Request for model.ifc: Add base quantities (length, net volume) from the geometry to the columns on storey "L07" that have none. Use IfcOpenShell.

First a look at what the model holds.

```python
import ifcopenshell
import ifcopenshell.util.element
import ifcopenshell.util.unit

model = ifcopenshell.open("model.ifc")
print(model.schema)
for unit_type in ("LENGTHUNIT", "AREAUNIT", "VOLUMEUNIT"):
    print(unit_type, ifcopenshell.util.unit.calculate_unit_scale(model, unit_type))
storey = next(s for s in model.by_type("IfcBuildingStorey") if s.Name == "L07")
columns = [e for e in ifcopenshell.util.element.get_decomposition(storey) if e.is_a("IfcColumn")]
for e in sorted(columns, key=lambda e: e.id()):
    print(e.id(), e.is_a(), e.Name, list(ifcopenshell.util.element.get_psets(e, qtos_only=True)), sep=" | ")
```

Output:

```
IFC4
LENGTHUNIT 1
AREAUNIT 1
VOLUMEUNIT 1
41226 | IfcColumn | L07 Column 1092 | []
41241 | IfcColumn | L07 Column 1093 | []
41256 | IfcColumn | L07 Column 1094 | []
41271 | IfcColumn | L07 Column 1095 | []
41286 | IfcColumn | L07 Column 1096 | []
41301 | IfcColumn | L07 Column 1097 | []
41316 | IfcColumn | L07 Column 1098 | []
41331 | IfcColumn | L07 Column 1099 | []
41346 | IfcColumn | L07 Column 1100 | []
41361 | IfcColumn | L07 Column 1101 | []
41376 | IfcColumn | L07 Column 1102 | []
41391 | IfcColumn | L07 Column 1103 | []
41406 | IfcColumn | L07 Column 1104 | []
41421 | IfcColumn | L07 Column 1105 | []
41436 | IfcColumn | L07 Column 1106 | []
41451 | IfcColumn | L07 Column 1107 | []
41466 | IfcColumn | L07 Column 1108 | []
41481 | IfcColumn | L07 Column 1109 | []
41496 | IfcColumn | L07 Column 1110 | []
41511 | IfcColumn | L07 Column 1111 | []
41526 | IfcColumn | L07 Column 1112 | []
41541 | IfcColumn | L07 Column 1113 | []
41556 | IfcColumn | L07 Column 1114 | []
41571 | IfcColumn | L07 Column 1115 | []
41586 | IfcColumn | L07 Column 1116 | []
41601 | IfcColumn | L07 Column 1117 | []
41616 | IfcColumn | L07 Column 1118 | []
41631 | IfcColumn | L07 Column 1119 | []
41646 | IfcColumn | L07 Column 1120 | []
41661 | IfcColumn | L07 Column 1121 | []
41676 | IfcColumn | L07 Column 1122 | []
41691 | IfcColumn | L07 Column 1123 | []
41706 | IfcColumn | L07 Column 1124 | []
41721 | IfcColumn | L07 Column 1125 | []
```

```python
import ifcopenshell
import ifcopenshell.api.pset
import ifcopenshell.geom
import ifcopenshell.util.element
import ifcopenshell.util.shape
import ifcopenshell.util.unit

model = ifcopenshell.open("model.ifc")
unit_scale = ifcopenshell.util.unit.calculate_unit_scale(model)
volume_scale = ifcopenshell.util.unit.calculate_unit_scale(model, "VOLUMEUNIT")
settings = ifcopenshell.geom.settings()

storey = next(s for s in model.by_type("IfcBuildingStorey") if s.Name == "L07")
columns = [e for e in ifcopenshell.util.element.get_decomposition(storey) if e.is_a("IfcColumn")]

for e in sorted(columns, key=lambda e: e.id()):
    if ifcopenshell.util.element.get_psets(e, qtos_only=True, should_inherit=False):
        continue
    # Geometry comes back in metres, in the element's own axes.
    shape = ifcopenshell.geom.create_shape(settings, e)
    values = {
        "Length": ifcopenshell.util.shape.get_z(shape.geometry) / unit_scale,
        "NetVolume": ifcopenshell.util.shape.get_volume(shape.geometry) / volume_scale,
    }
    qto = ifcopenshell.api.pset.add_qto(model, product=e, name="Qto_ColumnBaseQuantities")
    ifcopenshell.api.pset.edit_qto(model, qto=qto, properties=values)
    print(e.id(), {k: round(v, 3) for k, v in values.items()})

model.write("model_edited.ifc")
```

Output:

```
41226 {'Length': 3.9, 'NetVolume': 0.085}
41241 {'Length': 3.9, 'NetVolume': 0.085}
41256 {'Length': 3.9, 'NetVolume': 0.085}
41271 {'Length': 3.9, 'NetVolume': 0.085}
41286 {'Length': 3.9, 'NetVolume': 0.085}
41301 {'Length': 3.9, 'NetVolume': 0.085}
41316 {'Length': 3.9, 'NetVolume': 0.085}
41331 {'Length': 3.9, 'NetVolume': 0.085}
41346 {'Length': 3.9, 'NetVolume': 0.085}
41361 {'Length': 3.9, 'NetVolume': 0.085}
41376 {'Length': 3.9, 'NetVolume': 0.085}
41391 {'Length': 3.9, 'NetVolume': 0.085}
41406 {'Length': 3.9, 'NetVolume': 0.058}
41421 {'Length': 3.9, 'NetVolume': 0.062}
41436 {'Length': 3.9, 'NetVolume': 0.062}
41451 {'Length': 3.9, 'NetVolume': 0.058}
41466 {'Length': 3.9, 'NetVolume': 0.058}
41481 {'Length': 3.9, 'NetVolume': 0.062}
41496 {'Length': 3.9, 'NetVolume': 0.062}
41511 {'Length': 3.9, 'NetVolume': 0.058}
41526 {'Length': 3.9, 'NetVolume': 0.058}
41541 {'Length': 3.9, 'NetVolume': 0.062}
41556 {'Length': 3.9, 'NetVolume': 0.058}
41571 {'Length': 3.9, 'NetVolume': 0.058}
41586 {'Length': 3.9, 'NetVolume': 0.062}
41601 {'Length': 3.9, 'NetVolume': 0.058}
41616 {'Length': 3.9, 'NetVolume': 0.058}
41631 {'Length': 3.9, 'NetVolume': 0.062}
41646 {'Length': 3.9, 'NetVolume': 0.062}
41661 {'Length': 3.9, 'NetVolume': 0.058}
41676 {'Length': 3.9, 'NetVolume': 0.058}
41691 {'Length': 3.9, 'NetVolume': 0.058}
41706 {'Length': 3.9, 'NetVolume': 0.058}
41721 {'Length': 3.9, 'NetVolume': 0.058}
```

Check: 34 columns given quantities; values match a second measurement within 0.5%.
